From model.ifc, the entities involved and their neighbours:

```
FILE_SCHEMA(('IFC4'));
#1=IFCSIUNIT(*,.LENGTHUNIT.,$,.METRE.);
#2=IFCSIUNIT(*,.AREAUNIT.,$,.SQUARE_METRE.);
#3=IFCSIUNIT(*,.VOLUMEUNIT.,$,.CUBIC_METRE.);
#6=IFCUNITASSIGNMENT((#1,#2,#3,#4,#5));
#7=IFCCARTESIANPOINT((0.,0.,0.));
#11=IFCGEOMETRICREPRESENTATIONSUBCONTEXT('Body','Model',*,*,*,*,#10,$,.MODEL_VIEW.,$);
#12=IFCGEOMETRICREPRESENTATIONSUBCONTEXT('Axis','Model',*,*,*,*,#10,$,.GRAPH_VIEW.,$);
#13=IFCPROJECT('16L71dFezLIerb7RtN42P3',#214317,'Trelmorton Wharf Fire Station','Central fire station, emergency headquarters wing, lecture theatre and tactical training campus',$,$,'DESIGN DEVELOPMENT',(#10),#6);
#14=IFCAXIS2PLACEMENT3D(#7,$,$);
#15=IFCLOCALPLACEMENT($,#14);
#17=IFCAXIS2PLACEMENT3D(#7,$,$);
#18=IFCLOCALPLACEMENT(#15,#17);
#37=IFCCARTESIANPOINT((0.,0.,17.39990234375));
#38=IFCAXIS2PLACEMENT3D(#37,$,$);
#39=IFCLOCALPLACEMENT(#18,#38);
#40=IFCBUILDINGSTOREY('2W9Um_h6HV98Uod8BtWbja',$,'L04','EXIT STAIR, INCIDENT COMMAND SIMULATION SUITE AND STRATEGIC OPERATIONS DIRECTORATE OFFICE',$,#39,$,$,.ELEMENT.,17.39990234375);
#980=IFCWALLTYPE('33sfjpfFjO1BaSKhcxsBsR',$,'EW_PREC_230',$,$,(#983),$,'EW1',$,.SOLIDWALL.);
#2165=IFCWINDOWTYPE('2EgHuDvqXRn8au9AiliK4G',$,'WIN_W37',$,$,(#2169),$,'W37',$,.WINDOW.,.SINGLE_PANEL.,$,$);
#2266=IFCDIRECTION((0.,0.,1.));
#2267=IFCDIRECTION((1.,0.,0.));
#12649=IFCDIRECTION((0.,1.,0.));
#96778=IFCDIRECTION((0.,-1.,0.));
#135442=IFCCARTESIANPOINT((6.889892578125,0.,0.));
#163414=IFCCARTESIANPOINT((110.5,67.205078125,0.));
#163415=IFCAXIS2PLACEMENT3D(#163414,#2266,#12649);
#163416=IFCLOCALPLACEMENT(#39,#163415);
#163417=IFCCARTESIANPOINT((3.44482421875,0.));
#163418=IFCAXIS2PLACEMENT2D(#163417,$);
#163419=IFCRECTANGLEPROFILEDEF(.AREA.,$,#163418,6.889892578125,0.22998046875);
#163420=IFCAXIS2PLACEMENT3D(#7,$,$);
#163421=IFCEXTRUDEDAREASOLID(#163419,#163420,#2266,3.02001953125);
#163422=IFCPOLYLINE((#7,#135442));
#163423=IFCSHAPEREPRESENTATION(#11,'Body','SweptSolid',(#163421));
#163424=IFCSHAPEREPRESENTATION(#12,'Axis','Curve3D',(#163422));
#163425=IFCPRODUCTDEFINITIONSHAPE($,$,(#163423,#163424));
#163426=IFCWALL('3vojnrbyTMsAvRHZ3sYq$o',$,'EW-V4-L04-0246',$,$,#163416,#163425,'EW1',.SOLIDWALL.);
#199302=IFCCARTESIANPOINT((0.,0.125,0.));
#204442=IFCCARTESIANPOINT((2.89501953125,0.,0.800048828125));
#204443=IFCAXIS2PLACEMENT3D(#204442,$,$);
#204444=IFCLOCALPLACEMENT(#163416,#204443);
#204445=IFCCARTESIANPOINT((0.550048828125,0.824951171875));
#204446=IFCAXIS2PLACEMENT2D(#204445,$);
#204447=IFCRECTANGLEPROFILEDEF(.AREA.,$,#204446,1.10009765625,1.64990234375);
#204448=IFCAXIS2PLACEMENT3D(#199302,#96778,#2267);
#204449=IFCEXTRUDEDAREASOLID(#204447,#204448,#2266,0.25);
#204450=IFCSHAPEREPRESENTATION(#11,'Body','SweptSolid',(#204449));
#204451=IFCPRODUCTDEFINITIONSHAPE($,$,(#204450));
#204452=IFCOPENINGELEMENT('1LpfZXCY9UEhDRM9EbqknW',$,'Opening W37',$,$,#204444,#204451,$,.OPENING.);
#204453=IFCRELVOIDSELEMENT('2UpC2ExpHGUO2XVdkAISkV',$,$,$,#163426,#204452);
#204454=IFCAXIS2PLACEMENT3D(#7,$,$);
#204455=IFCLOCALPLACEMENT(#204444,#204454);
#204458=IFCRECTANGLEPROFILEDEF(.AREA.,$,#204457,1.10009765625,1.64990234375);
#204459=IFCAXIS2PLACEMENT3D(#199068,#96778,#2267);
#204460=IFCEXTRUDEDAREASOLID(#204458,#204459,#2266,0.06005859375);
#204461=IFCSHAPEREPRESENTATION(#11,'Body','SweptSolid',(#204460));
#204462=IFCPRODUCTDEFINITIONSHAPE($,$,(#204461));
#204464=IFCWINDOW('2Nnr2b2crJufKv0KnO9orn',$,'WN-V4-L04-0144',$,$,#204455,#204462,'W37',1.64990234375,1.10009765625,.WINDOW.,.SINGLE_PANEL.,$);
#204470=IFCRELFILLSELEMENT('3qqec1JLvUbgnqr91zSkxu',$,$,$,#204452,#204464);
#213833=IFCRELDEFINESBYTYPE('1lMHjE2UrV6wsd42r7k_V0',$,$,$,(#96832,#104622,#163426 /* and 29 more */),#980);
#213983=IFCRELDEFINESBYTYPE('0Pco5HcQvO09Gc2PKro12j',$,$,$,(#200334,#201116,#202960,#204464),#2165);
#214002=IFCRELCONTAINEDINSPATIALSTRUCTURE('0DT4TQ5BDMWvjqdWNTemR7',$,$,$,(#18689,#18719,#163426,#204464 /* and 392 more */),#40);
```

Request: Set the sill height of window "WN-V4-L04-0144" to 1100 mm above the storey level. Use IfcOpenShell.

```python
import numpy as np
import ifcopenshell
import ifcopenshell.api.geometry
import ifcopenshell.geom
import ifcopenshell.util.element
import ifcopenshell.util.placement
import ifcopenshell.util.shape
import ifcopenshell.util.unit

model = ifcopenshell.open("model.ifc")
unit_scale = ifcopenshell.util.unit.calculate_unit_scale(model)

window = model.by_id(204464)
opening = window.FillsVoids[0].RelatingOpeningElement
storey = ifcopenshell.util.element.get_container(window, ifc_class="IfcBuildingStorey")
level = ifcopenshell.util.placement.get_local_placement(storey.ObjectPlacement)[2, 3]

# The opening's origin need not be at the sill, so measure its lowest point.
shape = ifcopenshell.geom.create_shape(ifcopenshell.geom.settings(), opening)
bottom = ifcopenshell.util.shape.get_shape_bottom_elevation(shape, shape.geometry) / unit_scale
dz = level + 1.1 / unit_scale - bottom

shift = np.array([0.0, 0.0, dz])
# The window is placed relative to its opening, so it follows when the opening moves.
matrix = ifcopenshell.util.placement.get_local_placement(opening.ObjectPlacement)
matrix[:3, 3] += shift
ifcopenshell.api.geometry.edit_object_placement(
    model, product=opening, matrix=matrix, is_si=False, should_transform_children=True
)

print(f"moved by {dz * unit_scale:+.3f} m")

model.write("model_edited.ifc")
```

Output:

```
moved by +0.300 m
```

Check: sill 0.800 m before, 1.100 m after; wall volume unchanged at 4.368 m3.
